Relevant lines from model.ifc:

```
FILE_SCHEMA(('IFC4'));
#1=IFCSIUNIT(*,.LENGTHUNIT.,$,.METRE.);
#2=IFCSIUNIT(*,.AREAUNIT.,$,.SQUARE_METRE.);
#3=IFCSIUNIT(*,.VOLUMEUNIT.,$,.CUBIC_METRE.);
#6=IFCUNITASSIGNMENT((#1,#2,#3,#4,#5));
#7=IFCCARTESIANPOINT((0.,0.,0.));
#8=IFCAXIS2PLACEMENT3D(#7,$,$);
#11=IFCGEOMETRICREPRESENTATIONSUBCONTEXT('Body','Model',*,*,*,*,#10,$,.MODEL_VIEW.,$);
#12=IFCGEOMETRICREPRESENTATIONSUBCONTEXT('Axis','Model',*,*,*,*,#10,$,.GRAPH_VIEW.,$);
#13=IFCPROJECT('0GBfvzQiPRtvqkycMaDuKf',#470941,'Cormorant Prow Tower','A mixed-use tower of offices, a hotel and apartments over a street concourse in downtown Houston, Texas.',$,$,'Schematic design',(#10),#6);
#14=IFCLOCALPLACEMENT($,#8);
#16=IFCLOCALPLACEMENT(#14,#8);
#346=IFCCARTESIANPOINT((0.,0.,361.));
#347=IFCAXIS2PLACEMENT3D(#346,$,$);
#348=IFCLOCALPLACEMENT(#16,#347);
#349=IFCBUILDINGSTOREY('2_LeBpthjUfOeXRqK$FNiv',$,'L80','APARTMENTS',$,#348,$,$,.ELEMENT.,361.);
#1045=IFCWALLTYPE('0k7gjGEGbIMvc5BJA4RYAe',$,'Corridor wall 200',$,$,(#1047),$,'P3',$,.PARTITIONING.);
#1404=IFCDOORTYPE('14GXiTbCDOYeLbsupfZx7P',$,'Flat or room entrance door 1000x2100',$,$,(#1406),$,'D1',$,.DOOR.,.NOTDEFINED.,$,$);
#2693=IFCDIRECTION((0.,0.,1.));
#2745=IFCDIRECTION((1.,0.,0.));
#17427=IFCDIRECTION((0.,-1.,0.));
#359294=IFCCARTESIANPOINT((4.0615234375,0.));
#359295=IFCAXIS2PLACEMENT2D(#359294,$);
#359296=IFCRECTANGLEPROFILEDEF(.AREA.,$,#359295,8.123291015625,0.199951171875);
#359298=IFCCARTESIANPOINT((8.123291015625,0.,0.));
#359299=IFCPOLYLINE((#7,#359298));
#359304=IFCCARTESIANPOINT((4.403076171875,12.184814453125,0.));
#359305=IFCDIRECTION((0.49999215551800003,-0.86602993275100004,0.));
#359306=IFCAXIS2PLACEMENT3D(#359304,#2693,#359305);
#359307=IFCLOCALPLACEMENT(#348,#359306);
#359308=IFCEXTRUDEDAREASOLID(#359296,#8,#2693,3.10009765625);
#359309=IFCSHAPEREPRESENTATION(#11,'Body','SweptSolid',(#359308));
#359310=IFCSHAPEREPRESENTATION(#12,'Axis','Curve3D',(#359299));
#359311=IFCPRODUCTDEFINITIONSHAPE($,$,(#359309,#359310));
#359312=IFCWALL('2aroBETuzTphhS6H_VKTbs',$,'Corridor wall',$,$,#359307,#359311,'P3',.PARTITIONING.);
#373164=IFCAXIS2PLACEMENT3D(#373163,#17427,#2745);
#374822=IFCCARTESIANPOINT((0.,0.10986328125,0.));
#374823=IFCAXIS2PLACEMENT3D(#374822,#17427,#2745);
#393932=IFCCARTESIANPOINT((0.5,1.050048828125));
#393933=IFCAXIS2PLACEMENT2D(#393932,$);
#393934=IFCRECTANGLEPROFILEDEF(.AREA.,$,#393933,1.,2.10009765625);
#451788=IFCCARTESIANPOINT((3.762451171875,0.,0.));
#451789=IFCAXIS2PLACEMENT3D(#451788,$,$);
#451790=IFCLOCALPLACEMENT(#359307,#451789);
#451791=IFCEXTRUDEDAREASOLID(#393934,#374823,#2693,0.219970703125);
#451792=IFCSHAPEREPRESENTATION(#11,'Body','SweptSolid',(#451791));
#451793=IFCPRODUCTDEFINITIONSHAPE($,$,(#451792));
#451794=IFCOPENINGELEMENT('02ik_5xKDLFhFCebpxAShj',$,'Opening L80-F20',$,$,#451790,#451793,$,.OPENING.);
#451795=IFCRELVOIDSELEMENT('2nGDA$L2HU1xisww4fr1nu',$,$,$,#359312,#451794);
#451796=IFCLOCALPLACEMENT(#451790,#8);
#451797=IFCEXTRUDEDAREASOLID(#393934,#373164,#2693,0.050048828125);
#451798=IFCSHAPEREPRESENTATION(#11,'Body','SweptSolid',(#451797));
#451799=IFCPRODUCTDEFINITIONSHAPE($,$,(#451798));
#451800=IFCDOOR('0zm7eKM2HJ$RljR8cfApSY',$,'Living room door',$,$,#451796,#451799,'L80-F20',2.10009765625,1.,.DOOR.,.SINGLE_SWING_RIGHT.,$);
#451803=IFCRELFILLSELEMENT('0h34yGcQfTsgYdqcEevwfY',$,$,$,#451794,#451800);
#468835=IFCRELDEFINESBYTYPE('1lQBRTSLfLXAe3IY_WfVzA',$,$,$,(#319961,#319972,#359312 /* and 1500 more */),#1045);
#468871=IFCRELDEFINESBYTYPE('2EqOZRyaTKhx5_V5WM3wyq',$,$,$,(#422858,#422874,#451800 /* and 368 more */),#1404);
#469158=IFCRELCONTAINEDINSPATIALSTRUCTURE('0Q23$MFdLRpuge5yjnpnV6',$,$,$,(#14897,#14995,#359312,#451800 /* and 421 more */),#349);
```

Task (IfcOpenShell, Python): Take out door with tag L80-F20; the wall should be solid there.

```python
import ifcopenshell
import ifcopenshell.api.feature
import ifcopenshell.api.root
import ifcopenshell.geom
import ifcopenshell.util.shape

model = ifcopenshell.open("model.ifc")
settings = ifcopenshell.geom.settings()


def volume(element):
    """Net volume in cubic metres, openings subtracted."""
    shape = ifcopenshell.geom.create_shape(settings, element)
    return ifcopenshell.util.shape.get_volume(shape.geometry)


door = model.by_guid("0zm7eKM2HJ$RljR8cfApSY")
opening = door.FillsVoids[0].RelatingOpeningElement
wall = opening.VoidsElements[0].RelatingBuildingElement
before = volume(wall)

ifcopenshell.api.root.remove_product(model, product=door)
ifcopenshell.api.feature.remove_feature(model, feature=opening)

after = volume(wall)

print(f"wall volume {before:.3f} -> {after:.3f} m3")

model.write("model_edited.ifc")
```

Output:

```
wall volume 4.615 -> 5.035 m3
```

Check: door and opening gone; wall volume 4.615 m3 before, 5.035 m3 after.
